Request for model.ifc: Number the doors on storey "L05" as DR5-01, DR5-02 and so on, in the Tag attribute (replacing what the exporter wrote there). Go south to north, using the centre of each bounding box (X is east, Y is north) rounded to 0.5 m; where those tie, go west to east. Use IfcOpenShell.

First a look at what the model holds.

```python
import ifcopenshell
import ifcopenshell.util.element
import ifcopenshell.util.placement

model = ifcopenshell.open("model.ifc")
print(model.schema)
storey = next(s for s in model.by_type("IfcBuildingStorey") if s.Name == "L05")
doors = [e for e in ifcopenshell.util.element.get_decomposition(storey) if e.is_a("IfcDoor")]
for e in sorted(doors, key=lambda e: e.id()):
    origin = ifcopenshell.util.placement.get_local_placement(e.ObjectPlacement)[:3, 3]
    print(e.id(), e.Tag, e.Name, origin.round(2) + 0.0, sep=" | ")
```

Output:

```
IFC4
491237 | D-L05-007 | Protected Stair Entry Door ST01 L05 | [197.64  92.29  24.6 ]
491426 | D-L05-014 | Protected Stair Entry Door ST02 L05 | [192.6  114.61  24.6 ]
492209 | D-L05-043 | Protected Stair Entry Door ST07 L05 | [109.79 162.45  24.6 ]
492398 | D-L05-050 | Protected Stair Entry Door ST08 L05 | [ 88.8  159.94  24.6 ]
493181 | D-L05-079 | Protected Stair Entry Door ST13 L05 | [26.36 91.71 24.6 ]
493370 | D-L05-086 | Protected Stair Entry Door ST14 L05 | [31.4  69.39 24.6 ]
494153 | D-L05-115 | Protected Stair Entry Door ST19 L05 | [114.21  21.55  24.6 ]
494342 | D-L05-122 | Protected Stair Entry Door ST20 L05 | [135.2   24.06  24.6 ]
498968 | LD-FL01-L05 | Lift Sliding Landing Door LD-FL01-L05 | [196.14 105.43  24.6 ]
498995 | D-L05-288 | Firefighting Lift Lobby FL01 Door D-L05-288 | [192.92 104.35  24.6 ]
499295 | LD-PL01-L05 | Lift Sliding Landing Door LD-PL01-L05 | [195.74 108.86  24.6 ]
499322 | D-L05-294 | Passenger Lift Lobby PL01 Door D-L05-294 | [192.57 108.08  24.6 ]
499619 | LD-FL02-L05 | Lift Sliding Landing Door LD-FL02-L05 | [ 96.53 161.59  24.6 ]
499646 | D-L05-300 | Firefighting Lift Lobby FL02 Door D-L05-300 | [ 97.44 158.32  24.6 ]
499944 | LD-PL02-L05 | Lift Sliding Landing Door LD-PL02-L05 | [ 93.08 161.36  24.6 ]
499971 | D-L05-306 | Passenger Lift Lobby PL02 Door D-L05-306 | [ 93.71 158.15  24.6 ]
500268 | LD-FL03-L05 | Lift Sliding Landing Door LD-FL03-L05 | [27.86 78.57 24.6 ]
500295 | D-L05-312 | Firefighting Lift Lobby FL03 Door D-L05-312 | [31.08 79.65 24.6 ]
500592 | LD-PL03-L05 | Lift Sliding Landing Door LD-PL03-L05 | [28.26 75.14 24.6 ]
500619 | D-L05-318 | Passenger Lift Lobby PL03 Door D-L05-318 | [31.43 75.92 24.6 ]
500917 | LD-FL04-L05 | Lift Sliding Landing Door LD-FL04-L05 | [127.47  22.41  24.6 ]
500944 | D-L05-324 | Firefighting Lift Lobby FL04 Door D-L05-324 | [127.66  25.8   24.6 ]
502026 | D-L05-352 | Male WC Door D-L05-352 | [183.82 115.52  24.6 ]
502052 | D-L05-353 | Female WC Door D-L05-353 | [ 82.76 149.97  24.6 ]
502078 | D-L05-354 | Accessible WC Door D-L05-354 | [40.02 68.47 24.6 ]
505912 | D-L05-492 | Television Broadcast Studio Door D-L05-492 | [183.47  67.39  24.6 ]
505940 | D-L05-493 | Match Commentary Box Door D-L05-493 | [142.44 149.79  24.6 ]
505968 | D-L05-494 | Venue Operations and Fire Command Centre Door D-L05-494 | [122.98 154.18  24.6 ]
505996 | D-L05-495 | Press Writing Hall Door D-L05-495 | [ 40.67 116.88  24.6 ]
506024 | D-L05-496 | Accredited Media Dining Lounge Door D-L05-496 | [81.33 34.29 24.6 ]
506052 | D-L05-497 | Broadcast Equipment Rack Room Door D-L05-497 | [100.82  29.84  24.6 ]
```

```python
import ifcopenshell
import ifcopenshell.geom
import ifcopenshell.util.element
import ifcopenshell.util.shape

model = ifcopenshell.open("model.ifc")
settings = ifcopenshell.geom.settings()
settings.set("use-world-coords", True)


def centre(element):
    shape = ifcopenshell.geom.create_shape(settings, element)
    return ifcopenshell.util.shape.get_bbox_centroid(shape.geometry)


storey = next(s for s in model.by_type("IfcBuildingStorey") if s.Name == "L05")
doors = [e for e in ifcopenshell.util.element.get_decomposition(storey) if e.is_a("IfcDoor")]

# Insertion points can sit at a corner or the storey origin, so sort by the geometry (in metres).
centres = {e: centre(e) for e in doors}
doors.sort(key=lambda e: (round(centres[e][1] / 0.5), centres[e][0]))

for i, e in enumerate(doors, start=1):
    number = f"DR5-{i:02d}"
    e.Tag = number
    print(e.id(), number)

model.write("model-out.ifc")
```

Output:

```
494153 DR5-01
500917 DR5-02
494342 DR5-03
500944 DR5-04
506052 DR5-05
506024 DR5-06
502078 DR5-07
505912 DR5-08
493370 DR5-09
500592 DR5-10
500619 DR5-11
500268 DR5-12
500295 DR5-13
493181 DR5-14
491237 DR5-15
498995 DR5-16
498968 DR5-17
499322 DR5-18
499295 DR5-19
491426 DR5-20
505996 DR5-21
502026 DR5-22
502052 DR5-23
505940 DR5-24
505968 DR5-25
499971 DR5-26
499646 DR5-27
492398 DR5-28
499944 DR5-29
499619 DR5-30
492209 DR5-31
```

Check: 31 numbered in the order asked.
